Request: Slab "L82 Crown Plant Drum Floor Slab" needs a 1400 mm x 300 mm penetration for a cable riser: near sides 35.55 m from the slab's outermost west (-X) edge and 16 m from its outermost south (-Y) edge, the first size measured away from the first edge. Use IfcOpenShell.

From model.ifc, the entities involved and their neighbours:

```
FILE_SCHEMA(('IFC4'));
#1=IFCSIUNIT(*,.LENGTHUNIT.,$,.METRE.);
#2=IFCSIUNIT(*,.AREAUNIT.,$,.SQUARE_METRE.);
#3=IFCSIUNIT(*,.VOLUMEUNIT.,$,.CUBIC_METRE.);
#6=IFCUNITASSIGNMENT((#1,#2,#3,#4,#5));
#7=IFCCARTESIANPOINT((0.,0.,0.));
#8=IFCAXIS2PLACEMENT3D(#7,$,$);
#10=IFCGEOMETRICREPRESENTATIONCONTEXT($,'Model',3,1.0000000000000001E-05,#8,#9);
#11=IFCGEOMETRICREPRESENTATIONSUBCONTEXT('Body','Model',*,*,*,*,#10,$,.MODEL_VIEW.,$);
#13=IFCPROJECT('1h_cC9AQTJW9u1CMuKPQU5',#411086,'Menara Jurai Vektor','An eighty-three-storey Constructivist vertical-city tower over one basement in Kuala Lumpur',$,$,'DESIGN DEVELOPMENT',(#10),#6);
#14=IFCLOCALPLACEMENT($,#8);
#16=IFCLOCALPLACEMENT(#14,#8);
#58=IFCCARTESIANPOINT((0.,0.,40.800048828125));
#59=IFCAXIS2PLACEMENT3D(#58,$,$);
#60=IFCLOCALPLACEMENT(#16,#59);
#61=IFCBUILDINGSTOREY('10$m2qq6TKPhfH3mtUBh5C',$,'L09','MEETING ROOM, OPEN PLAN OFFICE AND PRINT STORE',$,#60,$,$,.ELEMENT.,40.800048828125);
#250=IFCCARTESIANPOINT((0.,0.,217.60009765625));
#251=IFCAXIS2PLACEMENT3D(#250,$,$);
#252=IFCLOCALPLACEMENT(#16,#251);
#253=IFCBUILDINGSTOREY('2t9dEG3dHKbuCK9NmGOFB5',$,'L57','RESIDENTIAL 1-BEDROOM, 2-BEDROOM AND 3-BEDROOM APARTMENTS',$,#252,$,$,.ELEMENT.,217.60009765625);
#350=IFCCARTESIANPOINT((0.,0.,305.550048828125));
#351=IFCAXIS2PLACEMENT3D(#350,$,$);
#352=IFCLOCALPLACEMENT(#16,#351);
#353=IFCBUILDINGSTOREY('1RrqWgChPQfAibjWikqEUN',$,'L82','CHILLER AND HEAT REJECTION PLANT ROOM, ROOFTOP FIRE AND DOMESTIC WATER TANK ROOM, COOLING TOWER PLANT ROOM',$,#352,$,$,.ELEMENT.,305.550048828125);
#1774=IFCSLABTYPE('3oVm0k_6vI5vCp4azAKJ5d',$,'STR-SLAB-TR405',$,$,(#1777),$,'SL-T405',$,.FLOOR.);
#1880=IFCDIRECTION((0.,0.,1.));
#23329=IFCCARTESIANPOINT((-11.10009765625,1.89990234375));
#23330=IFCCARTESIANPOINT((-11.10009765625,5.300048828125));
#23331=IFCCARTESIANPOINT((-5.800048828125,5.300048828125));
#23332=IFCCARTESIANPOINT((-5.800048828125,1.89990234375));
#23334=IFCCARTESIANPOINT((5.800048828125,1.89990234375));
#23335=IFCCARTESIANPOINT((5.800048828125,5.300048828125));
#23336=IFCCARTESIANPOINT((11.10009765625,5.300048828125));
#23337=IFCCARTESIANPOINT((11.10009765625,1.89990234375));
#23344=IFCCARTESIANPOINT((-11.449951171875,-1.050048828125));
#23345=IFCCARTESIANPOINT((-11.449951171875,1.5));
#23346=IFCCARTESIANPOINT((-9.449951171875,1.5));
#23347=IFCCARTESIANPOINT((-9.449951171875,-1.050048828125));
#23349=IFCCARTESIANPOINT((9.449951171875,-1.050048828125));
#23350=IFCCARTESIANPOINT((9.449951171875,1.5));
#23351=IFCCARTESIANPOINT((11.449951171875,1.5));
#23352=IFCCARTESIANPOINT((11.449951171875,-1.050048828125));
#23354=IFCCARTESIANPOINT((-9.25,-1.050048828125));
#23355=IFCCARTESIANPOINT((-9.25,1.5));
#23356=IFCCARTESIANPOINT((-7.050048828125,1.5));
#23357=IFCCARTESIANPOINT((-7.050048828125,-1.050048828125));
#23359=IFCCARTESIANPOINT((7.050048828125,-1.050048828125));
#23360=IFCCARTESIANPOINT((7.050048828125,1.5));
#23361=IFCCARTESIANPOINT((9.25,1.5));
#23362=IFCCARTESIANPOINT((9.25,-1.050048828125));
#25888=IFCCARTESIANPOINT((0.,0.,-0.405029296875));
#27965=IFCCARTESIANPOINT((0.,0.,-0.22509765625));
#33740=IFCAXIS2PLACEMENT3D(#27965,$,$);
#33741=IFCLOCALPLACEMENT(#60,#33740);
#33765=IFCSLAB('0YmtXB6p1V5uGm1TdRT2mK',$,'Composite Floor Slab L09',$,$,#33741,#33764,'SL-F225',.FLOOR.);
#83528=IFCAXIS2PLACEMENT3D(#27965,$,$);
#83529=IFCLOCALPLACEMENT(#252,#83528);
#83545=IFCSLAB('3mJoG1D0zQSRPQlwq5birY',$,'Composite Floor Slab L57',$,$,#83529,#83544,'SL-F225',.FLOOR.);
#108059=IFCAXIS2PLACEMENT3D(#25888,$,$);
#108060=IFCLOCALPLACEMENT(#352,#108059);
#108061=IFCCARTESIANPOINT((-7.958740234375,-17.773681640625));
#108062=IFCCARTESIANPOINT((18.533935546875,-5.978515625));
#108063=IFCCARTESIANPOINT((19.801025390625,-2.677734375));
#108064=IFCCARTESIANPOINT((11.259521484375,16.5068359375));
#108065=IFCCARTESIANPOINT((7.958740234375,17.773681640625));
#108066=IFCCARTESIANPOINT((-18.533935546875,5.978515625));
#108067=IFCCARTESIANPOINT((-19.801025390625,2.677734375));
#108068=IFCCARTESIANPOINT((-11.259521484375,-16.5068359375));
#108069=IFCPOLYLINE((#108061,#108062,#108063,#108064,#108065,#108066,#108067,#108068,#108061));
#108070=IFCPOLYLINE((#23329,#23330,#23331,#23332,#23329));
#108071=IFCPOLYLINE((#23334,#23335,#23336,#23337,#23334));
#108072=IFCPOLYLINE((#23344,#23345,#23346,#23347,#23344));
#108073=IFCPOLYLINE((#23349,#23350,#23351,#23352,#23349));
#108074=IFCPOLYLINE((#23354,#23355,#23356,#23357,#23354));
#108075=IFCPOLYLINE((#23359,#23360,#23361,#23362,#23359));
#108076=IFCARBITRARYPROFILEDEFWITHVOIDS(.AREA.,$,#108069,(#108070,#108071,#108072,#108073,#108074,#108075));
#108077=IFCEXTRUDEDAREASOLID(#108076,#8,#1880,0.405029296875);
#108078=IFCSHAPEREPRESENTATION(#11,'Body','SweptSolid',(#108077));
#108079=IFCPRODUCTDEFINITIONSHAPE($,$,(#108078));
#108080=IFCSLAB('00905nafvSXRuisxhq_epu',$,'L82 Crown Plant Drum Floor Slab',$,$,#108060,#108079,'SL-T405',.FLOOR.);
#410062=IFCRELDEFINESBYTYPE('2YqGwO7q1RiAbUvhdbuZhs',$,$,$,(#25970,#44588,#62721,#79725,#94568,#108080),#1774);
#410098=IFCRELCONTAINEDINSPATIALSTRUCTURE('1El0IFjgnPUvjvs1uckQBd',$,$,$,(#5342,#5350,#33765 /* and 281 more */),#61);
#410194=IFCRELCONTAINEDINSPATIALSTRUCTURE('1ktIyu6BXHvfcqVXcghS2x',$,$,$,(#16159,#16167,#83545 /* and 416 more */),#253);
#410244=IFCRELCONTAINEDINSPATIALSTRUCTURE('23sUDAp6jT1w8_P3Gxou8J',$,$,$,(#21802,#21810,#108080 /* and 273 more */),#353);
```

```python
import numpy as np
import ifcopenshell
import ifcopenshell.api.feature
import ifcopenshell.api.geometry
import ifcopenshell.api.root
import ifcopenshell.geom
import ifcopenshell.util.placement
import ifcopenshell.util.representation
import ifcopenshell.util.shape
import ifcopenshell.util.unit

model = ifcopenshell.open("model.ifc")
unit_scale = ifcopenshell.util.unit.calculate_unit_scale(model)
settings = ifcopenshell.geom.settings()


def volume(element):
    """Net volume in cubic metres, openings subtracted."""
    shape = ifcopenshell.geom.create_shape(settings, element)
    return ifcopenshell.util.shape.get_volume(shape.geometry)


slab = model.by_guid("00905nafvSXRuisxhq_epu")
before = volume(slab)

# Extent in the slab's own axes, in metres. The edges named are its -X and -Y sides.
slab_shape = ifcopenshell.geom.create_shape(settings, slab)
vertices = ifcopenshell.util.shape.get_vertices(slab_shape.geometry)
x_min, y_min, bottom = vertices.min(axis=0)
top = vertices[:, 2].max()

opening = ifcopenshell.api.root.create_entity(model, ifc_class="IfcOpeningElement", name="Cable riser opening", predefined_type="OPENING")
context = ifcopenshell.util.representation.get_context(model, "Model", "Body", "MODEL_VIEW")
width, depth = 1.4, 0.3
outline = [(0.0, 0.0), (width, 0.0), (width, depth), (0.0, depth), (0.0, 0.0)]
# Overshoot both faces by 50 mm so the cut is clean.
shape = ifcopenshell.api.geometry.add_slab_representation(
    model, context=context, depth=top - bottom + 0.1, polyline=outline
)
ifcopenshell.api.geometry.assign_representation(model, product=opening, representation=shape)

matrix = ifcopenshell.util.placement.get_local_placement(slab.ObjectPlacement)
matrix[:, 3] = matrix @ np.append(np.array([x_min + 35.55, y_min + 16, bottom - 0.05]) / unit_scale, 1.0)
ifcopenshell.api.geometry.edit_object_placement(model, product=opening, matrix=matrix, is_si=False)
ifcopenshell.api.feature.add_feature(model, feature=opening, element=slab)

after = volume(slab)

print(f"slab volume {before:.3f} -> {after:.3f} m3")

model.write("model_updated.ifc")
```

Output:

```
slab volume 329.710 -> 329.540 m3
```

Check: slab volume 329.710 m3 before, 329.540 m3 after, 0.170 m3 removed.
